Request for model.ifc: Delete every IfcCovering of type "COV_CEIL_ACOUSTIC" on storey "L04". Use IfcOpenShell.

First a look at what the model holds.

```python
import ifcopenshell
import ifcopenshell.util.element

model = ifcopenshell.open("model.ifc")
print(model.schema)
storey = next(s for s in model.by_type("IfcBuildingStorey") if s.Name == "L04")
coverings = [e for e in ifcopenshell.util.element.get_decomposition(storey) if e.is_a("IfcCovering")]
seen = {}
for e in coverings:
    element_type = ifcopenshell.util.element.get_type(e)
    name = element_type.Name if element_type not in (None, e) else None
    seen[name] = seen.get(name, 0) + 1
for name, count in sorted(seen.items(), key=str):
    print(count, "x", name)
```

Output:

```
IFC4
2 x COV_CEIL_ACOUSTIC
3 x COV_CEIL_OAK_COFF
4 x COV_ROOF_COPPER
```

```python
import ifcopenshell
import ifcopenshell.api.root
import ifcopenshell.util.element

model = ifcopenshell.open("model.ifc")

storey = next(s for s in model.by_type("IfcBuildingStorey") if s.Name == "L04")
coverings = [e for e in ifcopenshell.util.element.get_decomposition(storey) if e.is_a("IfcCovering")]
targets = [e for e in coverings if (t := ifcopenshell.util.element.get_type(e)) not in (None, e) and t.Name == "COV_CEIL_ACOUSTIC"]

for e in targets:
    ifcopenshell.api.root.remove_product(model, product=e)
print(len(targets), "removed")

model.write("model_rev.ifc")
```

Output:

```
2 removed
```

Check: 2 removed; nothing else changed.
